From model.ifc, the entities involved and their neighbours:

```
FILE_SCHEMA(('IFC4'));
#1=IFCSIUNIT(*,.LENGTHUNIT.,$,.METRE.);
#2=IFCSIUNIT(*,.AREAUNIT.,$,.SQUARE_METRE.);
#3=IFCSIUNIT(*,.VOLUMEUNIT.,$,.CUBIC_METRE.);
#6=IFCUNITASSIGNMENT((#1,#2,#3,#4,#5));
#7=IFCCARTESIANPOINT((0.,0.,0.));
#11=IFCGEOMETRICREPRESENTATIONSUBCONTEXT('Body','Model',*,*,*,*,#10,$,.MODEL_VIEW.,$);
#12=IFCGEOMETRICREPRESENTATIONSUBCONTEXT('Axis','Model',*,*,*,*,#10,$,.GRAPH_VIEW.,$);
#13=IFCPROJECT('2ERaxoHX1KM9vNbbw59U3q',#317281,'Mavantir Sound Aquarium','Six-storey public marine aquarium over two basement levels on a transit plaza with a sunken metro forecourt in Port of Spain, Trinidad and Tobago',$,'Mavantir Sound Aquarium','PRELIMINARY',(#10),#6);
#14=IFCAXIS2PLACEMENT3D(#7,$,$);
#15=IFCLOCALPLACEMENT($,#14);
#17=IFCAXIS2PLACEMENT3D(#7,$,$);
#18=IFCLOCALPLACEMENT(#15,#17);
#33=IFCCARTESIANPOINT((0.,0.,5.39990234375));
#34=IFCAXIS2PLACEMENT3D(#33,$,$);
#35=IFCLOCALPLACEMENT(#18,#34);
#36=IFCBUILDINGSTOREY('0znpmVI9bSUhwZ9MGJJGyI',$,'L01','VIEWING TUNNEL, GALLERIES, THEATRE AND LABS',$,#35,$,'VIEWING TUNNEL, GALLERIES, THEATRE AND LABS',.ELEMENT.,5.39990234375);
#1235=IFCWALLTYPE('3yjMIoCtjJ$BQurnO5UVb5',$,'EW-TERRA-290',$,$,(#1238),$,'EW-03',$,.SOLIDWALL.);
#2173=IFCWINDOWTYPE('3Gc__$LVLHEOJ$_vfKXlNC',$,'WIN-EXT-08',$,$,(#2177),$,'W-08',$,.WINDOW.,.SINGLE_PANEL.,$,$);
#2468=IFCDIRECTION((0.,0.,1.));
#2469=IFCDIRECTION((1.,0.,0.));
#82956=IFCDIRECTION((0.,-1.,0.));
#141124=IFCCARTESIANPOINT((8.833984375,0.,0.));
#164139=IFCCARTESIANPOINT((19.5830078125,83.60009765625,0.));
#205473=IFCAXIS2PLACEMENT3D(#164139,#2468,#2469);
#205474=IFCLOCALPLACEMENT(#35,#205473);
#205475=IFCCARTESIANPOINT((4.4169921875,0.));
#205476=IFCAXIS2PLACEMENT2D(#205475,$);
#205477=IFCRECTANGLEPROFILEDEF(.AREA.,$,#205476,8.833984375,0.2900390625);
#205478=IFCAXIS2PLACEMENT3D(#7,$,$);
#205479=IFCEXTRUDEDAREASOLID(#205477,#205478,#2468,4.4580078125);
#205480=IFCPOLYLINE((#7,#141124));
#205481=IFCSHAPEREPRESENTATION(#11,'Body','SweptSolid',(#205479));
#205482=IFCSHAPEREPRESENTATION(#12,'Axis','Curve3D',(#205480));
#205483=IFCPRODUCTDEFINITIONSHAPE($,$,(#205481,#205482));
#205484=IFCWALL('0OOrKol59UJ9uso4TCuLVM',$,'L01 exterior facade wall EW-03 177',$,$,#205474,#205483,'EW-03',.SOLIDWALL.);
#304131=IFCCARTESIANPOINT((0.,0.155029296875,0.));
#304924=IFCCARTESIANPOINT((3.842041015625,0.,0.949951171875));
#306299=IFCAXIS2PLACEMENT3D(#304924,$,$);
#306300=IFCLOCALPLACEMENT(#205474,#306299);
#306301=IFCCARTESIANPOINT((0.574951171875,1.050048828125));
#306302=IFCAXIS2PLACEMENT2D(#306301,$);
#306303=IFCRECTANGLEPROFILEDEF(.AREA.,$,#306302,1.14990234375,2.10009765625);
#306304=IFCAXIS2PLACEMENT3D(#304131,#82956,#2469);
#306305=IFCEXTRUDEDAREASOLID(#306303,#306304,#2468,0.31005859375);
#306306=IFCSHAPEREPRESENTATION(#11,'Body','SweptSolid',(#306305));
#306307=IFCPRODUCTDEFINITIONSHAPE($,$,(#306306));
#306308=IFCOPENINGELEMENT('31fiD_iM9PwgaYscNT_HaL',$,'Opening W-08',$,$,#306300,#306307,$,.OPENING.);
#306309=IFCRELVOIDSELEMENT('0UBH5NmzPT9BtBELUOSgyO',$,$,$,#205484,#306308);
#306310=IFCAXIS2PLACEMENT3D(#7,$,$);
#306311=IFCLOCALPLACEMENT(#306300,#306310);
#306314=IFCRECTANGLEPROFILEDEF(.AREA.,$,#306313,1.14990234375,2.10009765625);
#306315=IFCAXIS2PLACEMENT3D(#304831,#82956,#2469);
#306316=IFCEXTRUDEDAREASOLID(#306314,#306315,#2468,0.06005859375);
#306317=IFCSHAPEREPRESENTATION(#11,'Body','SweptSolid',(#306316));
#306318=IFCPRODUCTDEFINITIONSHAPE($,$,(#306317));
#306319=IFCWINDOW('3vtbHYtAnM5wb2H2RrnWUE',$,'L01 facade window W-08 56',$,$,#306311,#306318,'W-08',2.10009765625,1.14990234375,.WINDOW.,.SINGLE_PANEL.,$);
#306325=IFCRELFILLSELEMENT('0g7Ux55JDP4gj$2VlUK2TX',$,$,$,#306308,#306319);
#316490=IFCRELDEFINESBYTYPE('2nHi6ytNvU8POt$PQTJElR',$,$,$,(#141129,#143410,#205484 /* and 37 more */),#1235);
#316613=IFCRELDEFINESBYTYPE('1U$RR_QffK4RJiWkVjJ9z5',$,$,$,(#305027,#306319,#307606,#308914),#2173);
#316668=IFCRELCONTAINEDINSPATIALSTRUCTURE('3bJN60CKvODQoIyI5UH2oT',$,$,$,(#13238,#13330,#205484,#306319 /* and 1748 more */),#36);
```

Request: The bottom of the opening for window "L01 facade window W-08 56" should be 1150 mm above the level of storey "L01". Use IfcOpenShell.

```python
import numpy as np
import ifcopenshell
import ifcopenshell.api.geometry
import ifcopenshell.geom
import ifcopenshell.util.element
import ifcopenshell.util.placement
import ifcopenshell.util.shape
import ifcopenshell.util.unit

model = ifcopenshell.open("model.ifc")
unit_scale = ifcopenshell.util.unit.calculate_unit_scale(model)

window = model.by_guid("3vtbHYtAnM5wb2H2RrnWUE")
opening = window.FillsVoids[0].RelatingOpeningElement
storey = ifcopenshell.util.element.get_container(window, ifc_class="IfcBuildingStorey")
level = ifcopenshell.util.placement.get_local_placement(storey.ObjectPlacement)[2, 3]

# The opening's origin need not be at the sill, so measure its lowest point.
shape = ifcopenshell.geom.create_shape(ifcopenshell.geom.settings(), opening)
bottom = ifcopenshell.util.shape.get_shape_bottom_elevation(shape, shape.geometry) / unit_scale
dz = level + 1.15 - bottom

shift = np.array([0.0, 0.0, dz])
# The window is placed relative to its opening, so it follows when the opening moves.
matrix = ifcopenshell.util.placement.get_local_placement(opening.ObjectPlacement)
matrix[:3, 3] += shift
ifcopenshell.api.geometry.edit_object_placement(
    model, product=opening, matrix=matrix, is_si=False, should_transform_children=True
)

print(f"moved by {dz * unit_scale:+.3f} m")

model.write("model-out.ifc")
```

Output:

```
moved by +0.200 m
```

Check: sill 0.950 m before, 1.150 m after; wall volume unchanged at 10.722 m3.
